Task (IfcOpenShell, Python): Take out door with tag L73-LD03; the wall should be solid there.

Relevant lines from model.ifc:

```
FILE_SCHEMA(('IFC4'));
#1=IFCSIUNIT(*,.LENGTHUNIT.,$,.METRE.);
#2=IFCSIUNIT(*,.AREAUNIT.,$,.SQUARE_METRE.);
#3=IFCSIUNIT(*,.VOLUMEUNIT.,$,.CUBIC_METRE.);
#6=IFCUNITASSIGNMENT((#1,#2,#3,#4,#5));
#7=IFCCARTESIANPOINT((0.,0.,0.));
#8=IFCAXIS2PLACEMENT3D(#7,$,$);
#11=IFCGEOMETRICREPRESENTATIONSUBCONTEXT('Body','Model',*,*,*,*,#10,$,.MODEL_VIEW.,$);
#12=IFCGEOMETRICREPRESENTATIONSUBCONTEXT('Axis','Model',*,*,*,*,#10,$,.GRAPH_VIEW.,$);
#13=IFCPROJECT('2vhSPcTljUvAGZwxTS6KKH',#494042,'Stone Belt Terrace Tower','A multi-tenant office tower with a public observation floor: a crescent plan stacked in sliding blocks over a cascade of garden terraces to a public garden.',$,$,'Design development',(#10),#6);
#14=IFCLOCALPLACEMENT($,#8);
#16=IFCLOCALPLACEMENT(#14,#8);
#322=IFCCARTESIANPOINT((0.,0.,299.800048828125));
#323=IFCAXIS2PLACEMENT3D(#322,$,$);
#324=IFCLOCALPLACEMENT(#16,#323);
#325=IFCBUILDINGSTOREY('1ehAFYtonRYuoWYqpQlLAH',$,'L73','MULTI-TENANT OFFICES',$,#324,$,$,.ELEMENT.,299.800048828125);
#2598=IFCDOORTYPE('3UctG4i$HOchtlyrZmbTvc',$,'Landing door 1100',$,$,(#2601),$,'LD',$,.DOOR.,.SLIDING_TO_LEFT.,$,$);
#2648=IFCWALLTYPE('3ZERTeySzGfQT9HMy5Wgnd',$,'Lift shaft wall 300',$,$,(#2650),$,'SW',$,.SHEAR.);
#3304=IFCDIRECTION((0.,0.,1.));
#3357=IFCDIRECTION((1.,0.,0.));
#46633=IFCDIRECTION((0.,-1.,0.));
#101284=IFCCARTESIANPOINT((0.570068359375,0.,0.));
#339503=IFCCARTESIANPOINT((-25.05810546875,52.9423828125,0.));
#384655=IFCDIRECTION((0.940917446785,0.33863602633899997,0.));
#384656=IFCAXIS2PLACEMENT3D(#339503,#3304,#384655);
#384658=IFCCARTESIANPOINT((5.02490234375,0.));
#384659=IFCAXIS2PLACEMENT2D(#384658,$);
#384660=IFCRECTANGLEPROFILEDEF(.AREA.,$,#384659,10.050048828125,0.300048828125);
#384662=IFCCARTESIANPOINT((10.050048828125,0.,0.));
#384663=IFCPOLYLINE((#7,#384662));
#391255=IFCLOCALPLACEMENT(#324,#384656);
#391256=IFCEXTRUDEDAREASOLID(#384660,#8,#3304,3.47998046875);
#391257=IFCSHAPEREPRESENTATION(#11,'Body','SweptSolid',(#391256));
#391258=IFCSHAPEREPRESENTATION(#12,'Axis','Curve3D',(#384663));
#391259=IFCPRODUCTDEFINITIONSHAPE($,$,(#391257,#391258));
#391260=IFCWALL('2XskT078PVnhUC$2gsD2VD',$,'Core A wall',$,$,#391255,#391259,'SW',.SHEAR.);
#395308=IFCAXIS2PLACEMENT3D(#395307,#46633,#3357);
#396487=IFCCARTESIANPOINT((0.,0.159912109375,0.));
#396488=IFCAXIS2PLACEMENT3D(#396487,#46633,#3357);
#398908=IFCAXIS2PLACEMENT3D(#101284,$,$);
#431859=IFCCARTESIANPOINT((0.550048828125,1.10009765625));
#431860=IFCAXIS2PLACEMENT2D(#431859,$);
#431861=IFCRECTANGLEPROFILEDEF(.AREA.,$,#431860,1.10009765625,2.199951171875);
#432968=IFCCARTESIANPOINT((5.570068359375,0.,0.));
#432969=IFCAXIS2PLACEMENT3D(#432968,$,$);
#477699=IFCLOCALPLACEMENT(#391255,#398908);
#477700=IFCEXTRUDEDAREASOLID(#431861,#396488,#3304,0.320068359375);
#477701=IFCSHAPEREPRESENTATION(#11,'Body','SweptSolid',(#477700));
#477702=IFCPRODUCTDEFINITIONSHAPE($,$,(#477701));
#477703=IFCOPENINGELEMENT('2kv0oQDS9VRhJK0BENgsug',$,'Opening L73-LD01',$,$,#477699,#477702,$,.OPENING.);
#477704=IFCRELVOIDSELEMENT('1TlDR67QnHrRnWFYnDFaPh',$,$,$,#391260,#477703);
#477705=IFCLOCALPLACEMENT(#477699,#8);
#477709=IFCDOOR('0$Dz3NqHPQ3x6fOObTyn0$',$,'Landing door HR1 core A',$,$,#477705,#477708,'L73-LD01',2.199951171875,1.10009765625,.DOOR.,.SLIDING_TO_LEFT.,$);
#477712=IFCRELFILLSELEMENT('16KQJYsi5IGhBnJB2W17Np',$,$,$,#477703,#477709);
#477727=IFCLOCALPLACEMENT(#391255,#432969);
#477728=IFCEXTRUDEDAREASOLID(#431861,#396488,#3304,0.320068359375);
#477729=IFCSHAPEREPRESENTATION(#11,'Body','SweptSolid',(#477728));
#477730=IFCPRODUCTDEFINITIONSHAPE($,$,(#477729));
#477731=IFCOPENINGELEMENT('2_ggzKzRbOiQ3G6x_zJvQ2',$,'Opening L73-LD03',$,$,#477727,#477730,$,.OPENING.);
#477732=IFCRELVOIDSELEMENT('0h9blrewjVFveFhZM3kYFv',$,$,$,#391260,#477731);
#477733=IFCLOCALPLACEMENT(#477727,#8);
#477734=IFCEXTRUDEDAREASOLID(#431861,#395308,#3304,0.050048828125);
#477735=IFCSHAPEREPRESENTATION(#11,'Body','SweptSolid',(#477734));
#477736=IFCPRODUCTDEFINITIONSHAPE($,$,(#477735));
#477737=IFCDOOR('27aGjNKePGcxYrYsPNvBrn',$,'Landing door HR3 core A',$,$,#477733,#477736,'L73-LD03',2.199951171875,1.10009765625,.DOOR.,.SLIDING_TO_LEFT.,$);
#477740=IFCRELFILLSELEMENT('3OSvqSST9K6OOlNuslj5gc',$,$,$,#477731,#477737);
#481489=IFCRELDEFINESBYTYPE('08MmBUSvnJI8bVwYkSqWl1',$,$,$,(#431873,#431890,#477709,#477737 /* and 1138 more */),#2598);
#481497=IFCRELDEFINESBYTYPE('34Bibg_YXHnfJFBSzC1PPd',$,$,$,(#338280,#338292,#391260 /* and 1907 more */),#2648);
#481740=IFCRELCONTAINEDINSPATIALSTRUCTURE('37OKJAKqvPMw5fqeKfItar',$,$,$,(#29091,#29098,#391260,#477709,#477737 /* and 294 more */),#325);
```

```python
import ifcopenshell
import ifcopenshell.api.feature
import ifcopenshell.api.root
import ifcopenshell.geom
import ifcopenshell.util.shape

model = ifcopenshell.open("model.ifc")
settings = ifcopenshell.geom.settings()


def volume(element):
    """Net volume in cubic metres, openings subtracted."""
    shape = ifcopenshell.geom.create_shape(settings, element)
    return ifcopenshell.util.shape.get_volume(shape.geometry)


door = model.by_guid("27aGjNKePGcxYrYsPNvBrn")
opening = door.FillsVoids[0].RelatingOpeningElement
wall = opening.VoidsElements[0].RelatingBuildingElement
before = volume(wall)

ifcopenshell.api.root.remove_product(model, product=door)
ifcopenshell.api.feature.remove_feature(model, feature=opening)

after = volume(wall)

print(f"wall volume {before:.3f} -> {after:.3f} m3")

model.write("model_v2.ifc")
```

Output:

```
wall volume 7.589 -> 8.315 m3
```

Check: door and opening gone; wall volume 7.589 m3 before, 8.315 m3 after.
